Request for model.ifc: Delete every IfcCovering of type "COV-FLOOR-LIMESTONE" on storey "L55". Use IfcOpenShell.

First a look at what the model holds.

```python
import ifcopenshell
import ifcopenshell.util.element

model = ifcopenshell.open("model.ifc")
print(model.schema)
storey = next(s for s in model.by_type("IfcBuildingStorey") if s.Name == "L55")
coverings = [e for e in ifcopenshell.util.element.get_decomposition(storey) if e.is_a("IfcCovering")]
seen = {}
for e in coverings:
    element_type = ifcopenshell.util.element.get_type(e)
    name = element_type.Name if element_type not in (None, e) else None
    seen[name] = seen.get(name, 0) + 1
for name, count in sorted(seen.items(), key=str):
    print(count, "x", name)
```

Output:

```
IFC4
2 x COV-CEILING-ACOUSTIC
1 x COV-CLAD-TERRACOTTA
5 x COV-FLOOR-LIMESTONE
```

```python
import ifcopenshell
import ifcopenshell.api.root
import ifcopenshell.util.element

model = ifcopenshell.open("model.ifc")

storey = next(s for s in model.by_type("IfcBuildingStorey") if s.Name == "L55")
coverings = [e for e in ifcopenshell.util.element.get_decomposition(storey) if e.is_a("IfcCovering")]
targets = [e for e in coverings if (t := ifcopenshell.util.element.get_type(e)) not in (None, e) and t.Name == "COV-FLOOR-LIMESTONE"]

for e in targets:
    ifcopenshell.api.root.remove_product(model, product=e)
print(len(targets), "removed")

model.write("model_updated.ifc")
```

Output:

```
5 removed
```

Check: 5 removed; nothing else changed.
